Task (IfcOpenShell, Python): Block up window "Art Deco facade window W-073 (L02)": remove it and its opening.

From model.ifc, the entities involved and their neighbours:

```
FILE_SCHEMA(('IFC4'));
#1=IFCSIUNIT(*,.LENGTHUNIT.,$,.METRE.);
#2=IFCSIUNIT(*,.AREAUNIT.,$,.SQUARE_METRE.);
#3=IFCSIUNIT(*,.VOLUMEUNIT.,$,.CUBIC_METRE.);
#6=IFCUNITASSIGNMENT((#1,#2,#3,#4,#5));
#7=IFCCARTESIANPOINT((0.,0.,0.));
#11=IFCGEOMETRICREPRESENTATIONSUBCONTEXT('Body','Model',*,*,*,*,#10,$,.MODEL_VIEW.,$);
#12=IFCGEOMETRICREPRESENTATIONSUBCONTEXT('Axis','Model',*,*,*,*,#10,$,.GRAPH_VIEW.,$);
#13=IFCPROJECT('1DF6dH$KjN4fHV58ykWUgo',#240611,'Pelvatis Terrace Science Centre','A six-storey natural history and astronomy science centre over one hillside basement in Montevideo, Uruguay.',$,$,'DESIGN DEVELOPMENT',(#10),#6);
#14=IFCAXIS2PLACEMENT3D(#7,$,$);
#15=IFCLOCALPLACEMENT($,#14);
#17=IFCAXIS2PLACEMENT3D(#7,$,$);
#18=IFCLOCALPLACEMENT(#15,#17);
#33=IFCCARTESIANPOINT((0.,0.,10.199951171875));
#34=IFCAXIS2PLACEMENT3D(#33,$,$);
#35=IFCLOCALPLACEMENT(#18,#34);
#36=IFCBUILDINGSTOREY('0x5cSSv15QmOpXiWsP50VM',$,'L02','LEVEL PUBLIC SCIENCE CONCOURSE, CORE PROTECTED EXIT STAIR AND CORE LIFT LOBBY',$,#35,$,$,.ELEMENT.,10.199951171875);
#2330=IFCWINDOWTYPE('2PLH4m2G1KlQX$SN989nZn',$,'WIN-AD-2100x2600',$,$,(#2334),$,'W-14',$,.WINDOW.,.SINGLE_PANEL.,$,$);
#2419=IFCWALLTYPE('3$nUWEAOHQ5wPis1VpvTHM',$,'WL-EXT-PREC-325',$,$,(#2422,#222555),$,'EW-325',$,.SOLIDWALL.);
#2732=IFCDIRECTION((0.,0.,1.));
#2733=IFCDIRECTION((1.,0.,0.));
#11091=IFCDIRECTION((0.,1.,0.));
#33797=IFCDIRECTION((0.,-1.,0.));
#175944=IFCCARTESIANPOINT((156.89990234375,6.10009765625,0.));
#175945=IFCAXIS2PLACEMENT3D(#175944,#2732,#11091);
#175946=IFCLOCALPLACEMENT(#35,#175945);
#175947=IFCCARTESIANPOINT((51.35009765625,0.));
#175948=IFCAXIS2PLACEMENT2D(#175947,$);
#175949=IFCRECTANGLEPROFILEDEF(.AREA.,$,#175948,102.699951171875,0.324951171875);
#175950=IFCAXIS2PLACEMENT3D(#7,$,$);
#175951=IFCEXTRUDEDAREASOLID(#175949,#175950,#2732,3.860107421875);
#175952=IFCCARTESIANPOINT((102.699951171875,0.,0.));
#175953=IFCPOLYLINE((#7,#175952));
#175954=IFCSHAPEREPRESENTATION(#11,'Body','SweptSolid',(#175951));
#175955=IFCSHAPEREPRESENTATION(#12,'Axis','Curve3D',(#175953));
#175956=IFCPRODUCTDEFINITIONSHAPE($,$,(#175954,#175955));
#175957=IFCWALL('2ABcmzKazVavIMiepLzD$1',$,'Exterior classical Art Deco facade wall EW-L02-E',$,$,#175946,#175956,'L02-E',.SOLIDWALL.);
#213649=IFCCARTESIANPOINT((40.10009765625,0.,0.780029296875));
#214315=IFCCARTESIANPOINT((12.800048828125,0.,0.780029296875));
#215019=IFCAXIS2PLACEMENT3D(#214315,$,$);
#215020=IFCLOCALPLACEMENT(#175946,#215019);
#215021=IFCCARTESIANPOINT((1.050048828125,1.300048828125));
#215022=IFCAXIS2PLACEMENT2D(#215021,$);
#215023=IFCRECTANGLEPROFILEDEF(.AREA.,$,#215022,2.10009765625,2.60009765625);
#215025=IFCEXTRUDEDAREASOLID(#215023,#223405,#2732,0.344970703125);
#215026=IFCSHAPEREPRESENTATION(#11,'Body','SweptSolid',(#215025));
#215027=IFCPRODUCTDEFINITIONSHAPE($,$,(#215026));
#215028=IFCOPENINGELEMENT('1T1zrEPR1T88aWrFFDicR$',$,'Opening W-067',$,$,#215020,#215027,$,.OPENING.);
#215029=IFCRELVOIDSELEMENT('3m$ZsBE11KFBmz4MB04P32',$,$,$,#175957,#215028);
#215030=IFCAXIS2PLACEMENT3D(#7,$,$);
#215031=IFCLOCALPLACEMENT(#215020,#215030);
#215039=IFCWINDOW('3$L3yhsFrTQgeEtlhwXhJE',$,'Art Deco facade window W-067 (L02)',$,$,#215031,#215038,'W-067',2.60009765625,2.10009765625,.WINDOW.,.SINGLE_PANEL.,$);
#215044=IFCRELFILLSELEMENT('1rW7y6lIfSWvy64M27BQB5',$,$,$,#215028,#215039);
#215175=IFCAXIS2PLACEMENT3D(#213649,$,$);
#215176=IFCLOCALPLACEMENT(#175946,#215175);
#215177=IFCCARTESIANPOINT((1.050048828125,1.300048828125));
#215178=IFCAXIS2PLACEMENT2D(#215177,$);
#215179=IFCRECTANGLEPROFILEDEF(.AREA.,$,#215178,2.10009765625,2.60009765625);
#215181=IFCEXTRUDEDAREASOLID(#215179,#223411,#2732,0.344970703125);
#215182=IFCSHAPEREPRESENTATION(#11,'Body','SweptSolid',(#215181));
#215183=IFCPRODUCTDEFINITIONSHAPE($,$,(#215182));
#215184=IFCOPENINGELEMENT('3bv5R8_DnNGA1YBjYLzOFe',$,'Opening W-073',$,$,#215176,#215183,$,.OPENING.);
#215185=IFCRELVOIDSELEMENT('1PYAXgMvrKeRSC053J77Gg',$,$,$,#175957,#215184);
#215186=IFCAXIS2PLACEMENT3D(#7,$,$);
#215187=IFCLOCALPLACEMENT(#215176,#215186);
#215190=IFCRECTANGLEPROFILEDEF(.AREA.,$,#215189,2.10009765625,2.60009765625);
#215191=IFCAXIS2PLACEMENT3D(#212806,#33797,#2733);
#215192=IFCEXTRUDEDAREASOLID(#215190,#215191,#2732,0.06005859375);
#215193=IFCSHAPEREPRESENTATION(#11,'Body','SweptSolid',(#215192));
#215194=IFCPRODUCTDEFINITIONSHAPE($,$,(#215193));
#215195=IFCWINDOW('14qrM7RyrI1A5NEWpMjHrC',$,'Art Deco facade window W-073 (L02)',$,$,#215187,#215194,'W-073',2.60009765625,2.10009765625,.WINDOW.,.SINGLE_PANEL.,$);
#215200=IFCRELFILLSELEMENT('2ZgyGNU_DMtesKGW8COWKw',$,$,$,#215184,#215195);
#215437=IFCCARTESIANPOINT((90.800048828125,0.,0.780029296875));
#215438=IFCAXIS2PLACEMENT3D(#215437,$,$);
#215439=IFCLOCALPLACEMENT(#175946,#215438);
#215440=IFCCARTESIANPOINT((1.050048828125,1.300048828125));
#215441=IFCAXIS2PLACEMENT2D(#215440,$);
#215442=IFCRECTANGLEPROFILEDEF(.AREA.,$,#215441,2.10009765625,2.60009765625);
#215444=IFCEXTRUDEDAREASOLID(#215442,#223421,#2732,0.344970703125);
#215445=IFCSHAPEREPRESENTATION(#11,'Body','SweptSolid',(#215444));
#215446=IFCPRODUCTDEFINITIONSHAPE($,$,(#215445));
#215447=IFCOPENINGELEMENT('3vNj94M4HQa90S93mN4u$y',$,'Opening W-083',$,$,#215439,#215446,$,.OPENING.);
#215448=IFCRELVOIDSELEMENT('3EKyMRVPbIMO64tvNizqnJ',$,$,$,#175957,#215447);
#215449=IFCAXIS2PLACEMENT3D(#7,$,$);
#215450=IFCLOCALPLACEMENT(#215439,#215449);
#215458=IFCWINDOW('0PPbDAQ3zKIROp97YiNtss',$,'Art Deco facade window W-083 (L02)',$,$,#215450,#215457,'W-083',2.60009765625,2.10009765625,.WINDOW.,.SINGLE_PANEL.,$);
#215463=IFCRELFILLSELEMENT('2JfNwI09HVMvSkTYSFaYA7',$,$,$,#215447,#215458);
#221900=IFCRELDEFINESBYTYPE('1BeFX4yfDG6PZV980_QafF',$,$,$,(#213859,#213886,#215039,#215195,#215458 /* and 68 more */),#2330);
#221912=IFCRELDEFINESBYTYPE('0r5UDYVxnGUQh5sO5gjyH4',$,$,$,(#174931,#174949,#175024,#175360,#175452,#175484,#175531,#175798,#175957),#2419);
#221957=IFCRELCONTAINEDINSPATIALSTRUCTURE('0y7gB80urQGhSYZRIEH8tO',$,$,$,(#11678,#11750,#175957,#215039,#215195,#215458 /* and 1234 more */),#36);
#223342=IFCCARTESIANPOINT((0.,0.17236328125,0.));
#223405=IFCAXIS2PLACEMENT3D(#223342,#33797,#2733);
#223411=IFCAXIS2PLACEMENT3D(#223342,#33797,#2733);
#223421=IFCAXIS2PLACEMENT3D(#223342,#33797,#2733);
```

```python
import ifcopenshell
import ifcopenshell.api.feature
import ifcopenshell.api.root
import ifcopenshell.geom
import ifcopenshell.util.shape

model = ifcopenshell.open("model.ifc")
settings = ifcopenshell.geom.settings()


def volume(element):
    """Net volume in cubic metres, openings subtracted."""
    shape = ifcopenshell.geom.create_shape(settings, element)
    return ifcopenshell.util.shape.get_volume(shape.geometry)


window = model.by_id(215195)
opening = window.FillsVoids[0].RelatingOpeningElement
wall = opening.VoidsElements[0].RelatingBuildingElement
before = volume(wall)

ifcopenshell.api.root.remove_product(model, product=window)
ifcopenshell.api.feature.remove_feature(model, feature=opening)

after = volume(wall)

print(f"wall volume {before:.3f} -> {after:.3f} m3")

model.write("model_rev.ifc")
```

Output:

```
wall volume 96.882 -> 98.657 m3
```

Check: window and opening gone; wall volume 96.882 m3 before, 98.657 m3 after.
